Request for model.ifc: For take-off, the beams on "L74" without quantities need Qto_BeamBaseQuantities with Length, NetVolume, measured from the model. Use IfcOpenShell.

First a look at what the model holds.

```python
import ifcopenshell
import ifcopenshell.util.element
import ifcopenshell.util.unit

model = ifcopenshell.open("model.ifc")
print(model.schema)
for unit_type in ("LENGTHUNIT", "AREAUNIT", "VOLUMEUNIT"):
    print(unit_type, ifcopenshell.util.unit.calculate_unit_scale(model, unit_type))
storey = next(s for s in model.by_type("IfcBuildingStorey") if s.Name == "L74")
beams = [e for e in ifcopenshell.util.element.get_decomposition(storey) if e.is_a("IfcBeam")]
for e in sorted(beams, key=lambda e: e.id()):
    print(e.id(), e.is_a(), e.Name, list(ifcopenshell.util.element.get_psets(e, qtos_only=True)), sep=" | ")
```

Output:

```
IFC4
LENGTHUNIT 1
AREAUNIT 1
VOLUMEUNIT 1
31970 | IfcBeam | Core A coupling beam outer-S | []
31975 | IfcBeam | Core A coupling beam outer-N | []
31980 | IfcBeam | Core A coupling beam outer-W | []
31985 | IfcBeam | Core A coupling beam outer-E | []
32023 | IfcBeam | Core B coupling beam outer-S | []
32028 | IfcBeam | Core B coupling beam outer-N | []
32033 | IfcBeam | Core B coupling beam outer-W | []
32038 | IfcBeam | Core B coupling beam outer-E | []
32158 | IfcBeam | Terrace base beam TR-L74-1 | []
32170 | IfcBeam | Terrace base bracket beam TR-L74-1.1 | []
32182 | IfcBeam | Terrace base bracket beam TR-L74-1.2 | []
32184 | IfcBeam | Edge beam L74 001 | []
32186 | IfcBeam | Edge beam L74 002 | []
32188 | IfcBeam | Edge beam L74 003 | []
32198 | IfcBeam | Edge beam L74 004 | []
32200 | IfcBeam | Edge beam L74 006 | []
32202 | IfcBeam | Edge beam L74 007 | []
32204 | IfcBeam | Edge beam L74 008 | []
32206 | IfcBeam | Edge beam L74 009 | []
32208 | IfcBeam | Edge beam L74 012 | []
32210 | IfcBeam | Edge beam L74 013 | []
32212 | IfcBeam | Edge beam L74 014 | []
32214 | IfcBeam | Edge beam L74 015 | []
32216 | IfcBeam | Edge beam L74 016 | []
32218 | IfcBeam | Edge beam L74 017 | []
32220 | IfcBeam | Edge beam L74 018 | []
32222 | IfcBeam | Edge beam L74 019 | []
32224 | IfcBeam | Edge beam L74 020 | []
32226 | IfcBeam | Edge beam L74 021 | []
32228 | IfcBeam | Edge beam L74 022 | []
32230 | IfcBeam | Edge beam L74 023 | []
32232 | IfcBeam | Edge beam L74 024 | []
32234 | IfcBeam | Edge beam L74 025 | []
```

```python
import ifcopenshell
import ifcopenshell.api.pset
import ifcopenshell.geom
import ifcopenshell.util.element
import ifcopenshell.util.shape
import ifcopenshell.util.unit

model = ifcopenshell.open("model.ifc")
unit_scale = ifcopenshell.util.unit.calculate_unit_scale(model)
volume_scale = ifcopenshell.util.unit.calculate_unit_scale(model, "VOLUMEUNIT")
settings = ifcopenshell.geom.settings()

storey = next(s for s in model.by_type("IfcBuildingStorey") if s.Name == "L74")
beams = [e for e in ifcopenshell.util.element.get_decomposition(storey) if e.is_a("IfcBeam")]

for e in sorted(beams, key=lambda e: e.id()):
    if ifcopenshell.util.element.get_psets(e, qtos_only=True, should_inherit=False):
        continue
    # Geometry comes back in metres, in the element's own axes.
    shape = ifcopenshell.geom.create_shape(settings, e)
    values = {
        "Length": ifcopenshell.util.shape.get_max_xyz(shape.geometry) / unit_scale,
        "NetVolume": ifcopenshell.util.shape.get_volume(shape.geometry) / volume_scale,
    }
    qto = ifcopenshell.api.pset.add_qto(model, product=e, name="Qto_BeamBaseQuantities")
    ifcopenshell.api.pset.edit_qto(model, qto=qto, properties=values)
    print(e.id(), {k: round(v, 3) for k, v in values.items()})

model.write("model_updated.ifc")
```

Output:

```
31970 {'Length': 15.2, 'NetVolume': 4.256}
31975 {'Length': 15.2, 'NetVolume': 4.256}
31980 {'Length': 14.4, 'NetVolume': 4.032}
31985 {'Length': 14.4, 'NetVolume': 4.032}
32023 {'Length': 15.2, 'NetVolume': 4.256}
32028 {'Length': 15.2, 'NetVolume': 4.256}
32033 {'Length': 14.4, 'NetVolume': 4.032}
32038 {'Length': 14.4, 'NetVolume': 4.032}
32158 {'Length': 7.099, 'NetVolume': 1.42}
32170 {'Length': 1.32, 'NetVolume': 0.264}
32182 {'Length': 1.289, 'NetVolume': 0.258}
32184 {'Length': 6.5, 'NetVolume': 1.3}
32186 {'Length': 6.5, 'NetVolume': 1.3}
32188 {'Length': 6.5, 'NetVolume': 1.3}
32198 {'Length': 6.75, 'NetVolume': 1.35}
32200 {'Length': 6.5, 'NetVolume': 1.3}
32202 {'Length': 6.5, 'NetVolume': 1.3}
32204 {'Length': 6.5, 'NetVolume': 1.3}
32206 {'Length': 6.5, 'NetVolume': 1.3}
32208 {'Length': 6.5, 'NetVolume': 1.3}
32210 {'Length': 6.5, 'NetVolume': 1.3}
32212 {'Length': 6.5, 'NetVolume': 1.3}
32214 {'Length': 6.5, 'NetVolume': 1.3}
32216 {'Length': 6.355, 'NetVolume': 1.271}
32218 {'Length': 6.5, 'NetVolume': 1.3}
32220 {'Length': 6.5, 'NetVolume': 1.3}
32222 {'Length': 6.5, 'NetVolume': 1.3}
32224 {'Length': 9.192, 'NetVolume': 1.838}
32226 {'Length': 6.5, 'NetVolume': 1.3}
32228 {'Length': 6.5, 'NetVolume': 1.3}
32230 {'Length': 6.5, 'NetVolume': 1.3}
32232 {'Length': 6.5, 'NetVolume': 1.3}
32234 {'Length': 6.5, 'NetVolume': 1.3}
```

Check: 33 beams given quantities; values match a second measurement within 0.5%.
